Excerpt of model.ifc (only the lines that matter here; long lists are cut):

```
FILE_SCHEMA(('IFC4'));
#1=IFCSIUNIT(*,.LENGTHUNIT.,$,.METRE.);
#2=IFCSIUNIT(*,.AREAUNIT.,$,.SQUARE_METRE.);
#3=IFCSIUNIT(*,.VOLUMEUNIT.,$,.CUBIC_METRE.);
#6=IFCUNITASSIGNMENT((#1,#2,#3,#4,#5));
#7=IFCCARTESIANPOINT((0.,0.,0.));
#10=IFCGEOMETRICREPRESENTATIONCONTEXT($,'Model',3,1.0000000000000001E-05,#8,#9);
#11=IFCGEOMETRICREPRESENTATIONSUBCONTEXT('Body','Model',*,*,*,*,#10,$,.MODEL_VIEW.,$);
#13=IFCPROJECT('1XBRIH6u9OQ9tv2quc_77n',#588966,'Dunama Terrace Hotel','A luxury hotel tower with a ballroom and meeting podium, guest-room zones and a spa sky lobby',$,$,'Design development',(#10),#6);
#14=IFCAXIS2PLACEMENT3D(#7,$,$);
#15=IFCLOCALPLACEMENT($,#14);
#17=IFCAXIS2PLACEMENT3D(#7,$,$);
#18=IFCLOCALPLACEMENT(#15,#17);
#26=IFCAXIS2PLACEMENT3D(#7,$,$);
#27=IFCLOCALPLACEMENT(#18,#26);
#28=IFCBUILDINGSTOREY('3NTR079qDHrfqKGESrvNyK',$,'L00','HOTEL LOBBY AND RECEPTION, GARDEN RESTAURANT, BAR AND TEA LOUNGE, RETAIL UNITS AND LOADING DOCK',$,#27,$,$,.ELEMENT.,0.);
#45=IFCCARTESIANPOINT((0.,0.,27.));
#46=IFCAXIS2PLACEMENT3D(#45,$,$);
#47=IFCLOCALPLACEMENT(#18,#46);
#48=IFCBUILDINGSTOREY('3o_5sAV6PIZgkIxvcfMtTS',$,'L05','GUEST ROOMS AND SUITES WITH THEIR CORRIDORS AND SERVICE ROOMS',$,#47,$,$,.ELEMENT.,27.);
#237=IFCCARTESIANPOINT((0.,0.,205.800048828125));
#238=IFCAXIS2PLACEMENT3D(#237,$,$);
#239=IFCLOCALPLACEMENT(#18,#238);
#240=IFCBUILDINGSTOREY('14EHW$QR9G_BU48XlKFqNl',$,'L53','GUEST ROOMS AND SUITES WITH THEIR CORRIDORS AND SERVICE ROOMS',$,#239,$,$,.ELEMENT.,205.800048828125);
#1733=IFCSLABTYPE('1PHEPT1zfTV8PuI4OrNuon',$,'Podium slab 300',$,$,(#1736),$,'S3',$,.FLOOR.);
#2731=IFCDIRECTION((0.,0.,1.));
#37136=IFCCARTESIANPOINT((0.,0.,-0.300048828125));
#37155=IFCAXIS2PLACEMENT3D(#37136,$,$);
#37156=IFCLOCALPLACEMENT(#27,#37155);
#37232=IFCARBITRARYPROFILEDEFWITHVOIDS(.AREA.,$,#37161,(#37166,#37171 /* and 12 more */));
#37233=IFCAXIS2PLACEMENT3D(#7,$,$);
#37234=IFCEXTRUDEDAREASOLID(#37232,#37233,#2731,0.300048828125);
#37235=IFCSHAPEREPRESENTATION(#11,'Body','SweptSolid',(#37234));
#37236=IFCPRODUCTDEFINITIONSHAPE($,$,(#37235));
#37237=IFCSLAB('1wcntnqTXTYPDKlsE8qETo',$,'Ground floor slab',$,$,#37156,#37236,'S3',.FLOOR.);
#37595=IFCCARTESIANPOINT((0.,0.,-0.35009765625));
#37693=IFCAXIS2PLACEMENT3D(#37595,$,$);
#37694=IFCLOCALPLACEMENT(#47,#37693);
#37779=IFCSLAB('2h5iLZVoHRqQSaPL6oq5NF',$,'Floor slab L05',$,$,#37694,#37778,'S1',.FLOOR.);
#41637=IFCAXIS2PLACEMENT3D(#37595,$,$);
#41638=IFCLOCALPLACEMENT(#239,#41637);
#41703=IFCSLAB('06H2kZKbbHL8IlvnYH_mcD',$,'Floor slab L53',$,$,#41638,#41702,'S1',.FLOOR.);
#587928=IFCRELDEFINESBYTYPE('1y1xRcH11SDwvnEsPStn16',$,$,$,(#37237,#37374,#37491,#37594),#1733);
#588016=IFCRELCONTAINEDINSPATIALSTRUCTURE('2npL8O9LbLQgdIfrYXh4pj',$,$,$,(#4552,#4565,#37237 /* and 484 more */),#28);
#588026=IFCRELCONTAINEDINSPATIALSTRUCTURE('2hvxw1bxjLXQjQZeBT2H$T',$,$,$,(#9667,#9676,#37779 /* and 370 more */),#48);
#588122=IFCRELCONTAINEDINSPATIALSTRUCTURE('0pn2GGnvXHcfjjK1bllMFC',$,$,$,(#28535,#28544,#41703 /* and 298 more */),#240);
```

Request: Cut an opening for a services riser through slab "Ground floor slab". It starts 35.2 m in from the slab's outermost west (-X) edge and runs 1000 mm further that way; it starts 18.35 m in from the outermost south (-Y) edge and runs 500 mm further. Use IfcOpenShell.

```python
import numpy as np
import ifcopenshell
import ifcopenshell.api.feature
import ifcopenshell.api.geometry
import ifcopenshell.api.root
import ifcopenshell.geom
import ifcopenshell.util.placement
import ifcopenshell.util.representation
import ifcopenshell.util.shape
import ifcopenshell.util.unit

model = ifcopenshell.open("model.ifc")
unit_scale = ifcopenshell.util.unit.calculate_unit_scale(model)
settings = ifcopenshell.geom.settings()


def volume(element):
    """Net volume in cubic metres, openings subtracted."""
    shape = ifcopenshell.geom.create_shape(settings, element)
    return ifcopenshell.util.shape.get_volume(shape.geometry)


slab = model.by_guid("1wcntnqTXTYPDKlsE8qETo")
before = volume(slab)

# Extent in the slab's own axes, in metres. The edges named are its -X and -Y sides.
slab_shape = ifcopenshell.geom.create_shape(settings, slab)
vertices = ifcopenshell.util.shape.get_vertices(slab_shape.geometry)
x_min, y_min, bottom = vertices.min(axis=0)
top = vertices[:, 2].max()

opening = ifcopenshell.api.root.create_entity(model, ifc_class="IfcOpeningElement", name="Services riser opening", predefined_type="OPENING")
context = ifcopenshell.util.representation.get_context(model, "Model", "Body", "MODEL_VIEW")
width, depth = 1, 0.5
outline = [(0.0, 0.0), (width, 0.0), (width, depth), (0.0, depth), (0.0, 0.0)]
# Overshoot both faces by 50 mm so the cut is clean.
shape = ifcopenshell.api.geometry.add_slab_representation(
    model, context=context, depth=top - bottom + 0.1, polyline=outline
)
ifcopenshell.api.geometry.assign_representation(model, product=opening, representation=shape)

matrix = ifcopenshell.util.placement.get_local_placement(slab.ObjectPlacement)
matrix[:, 3] = matrix @ np.append(np.array([x_min + 35.2, y_min + 18.35, bottom - 0.05]) / unit_scale, 1.0)
ifcopenshell.api.geometry.edit_object_placement(model, product=opening, matrix=matrix, is_si=False)
ifcopenshell.api.feature.add_feature(model, feature=opening, element=slab)

after = volume(slab)

print(f"slab volume {before:.3f} -> {after:.3f} m3")

model.write("model_updated.ifc")
```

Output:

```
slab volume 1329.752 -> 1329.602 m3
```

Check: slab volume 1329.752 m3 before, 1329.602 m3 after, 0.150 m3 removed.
